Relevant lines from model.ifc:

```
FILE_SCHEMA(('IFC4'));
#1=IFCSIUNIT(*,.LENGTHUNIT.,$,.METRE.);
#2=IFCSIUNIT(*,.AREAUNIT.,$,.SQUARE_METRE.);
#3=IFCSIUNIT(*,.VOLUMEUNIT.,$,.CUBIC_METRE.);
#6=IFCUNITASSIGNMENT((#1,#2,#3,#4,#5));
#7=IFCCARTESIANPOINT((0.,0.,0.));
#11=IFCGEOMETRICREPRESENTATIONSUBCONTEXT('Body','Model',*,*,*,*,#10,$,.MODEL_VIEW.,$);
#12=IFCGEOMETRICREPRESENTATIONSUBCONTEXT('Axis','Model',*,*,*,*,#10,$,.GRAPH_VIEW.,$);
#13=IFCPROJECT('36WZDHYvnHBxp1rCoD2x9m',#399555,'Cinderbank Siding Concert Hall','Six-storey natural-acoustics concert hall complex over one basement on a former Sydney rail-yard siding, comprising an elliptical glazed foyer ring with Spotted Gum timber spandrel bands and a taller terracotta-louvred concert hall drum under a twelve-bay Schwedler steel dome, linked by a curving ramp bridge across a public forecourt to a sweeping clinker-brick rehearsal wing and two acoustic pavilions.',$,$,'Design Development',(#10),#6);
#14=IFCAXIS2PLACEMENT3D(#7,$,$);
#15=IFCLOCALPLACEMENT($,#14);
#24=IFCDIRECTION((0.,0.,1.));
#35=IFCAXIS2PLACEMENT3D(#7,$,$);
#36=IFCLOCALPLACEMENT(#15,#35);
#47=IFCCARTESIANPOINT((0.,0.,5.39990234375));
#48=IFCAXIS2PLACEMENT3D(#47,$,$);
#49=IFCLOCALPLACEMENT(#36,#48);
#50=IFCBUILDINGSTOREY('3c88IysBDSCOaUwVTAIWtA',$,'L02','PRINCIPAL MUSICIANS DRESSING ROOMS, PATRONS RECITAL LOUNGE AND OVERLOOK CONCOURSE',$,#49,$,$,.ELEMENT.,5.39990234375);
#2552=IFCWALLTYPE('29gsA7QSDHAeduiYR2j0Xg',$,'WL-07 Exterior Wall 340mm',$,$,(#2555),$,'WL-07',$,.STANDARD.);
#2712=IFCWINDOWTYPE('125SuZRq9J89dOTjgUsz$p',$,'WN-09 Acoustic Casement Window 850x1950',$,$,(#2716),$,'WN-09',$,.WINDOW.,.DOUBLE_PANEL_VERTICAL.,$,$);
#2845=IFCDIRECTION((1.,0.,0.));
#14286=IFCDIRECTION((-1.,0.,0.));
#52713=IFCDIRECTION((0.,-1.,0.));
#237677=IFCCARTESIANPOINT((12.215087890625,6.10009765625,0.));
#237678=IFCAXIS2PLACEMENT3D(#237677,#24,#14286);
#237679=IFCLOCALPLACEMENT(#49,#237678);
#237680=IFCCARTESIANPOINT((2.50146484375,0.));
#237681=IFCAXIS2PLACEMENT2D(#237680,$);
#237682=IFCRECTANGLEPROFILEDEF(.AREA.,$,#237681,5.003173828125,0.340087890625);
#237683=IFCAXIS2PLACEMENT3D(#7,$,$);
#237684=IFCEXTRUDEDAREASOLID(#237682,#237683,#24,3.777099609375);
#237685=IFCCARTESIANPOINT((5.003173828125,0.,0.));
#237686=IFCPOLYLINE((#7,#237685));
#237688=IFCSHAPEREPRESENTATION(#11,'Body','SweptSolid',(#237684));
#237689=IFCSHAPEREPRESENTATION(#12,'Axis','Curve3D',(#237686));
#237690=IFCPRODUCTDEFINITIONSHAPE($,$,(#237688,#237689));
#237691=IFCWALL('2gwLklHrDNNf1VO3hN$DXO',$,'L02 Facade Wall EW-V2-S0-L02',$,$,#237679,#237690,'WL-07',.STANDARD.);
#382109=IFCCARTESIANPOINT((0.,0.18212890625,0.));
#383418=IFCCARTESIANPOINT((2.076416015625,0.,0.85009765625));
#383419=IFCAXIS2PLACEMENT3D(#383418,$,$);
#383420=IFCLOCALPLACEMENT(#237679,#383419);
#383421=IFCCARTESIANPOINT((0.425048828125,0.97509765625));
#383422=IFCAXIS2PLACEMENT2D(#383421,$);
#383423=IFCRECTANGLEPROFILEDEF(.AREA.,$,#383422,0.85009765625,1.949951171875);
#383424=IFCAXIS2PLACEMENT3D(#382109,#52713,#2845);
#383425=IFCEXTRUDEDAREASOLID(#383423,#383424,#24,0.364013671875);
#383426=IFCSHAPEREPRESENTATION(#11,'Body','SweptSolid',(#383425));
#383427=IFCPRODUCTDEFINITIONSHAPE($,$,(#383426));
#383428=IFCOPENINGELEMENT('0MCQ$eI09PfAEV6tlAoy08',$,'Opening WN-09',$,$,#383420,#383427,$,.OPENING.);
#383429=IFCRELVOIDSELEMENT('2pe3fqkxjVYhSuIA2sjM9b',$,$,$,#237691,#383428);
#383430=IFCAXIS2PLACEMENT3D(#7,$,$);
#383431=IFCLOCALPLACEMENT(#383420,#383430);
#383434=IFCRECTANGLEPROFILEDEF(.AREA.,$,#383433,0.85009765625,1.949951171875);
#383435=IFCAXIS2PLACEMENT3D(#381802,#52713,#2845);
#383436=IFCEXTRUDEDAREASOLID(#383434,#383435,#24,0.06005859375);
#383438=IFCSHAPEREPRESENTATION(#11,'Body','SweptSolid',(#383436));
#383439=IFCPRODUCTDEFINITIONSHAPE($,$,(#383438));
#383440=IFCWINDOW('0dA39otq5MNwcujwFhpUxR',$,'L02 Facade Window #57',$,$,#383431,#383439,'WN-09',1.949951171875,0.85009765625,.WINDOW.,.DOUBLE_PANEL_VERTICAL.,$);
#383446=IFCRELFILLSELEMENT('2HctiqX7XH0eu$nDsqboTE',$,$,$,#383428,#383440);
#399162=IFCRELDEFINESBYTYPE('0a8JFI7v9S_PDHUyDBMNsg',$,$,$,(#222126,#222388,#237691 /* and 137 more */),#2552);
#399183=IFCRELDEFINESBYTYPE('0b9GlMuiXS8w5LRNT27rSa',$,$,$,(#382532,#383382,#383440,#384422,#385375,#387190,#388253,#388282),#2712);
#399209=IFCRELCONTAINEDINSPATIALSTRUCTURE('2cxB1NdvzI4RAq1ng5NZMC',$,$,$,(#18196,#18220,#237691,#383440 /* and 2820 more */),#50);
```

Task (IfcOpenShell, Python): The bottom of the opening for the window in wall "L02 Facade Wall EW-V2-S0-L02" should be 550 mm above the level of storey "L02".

```python
import numpy as np
import ifcopenshell
import ifcopenshell.api.geometry
import ifcopenshell.geom
import ifcopenshell.util.element
import ifcopenshell.util.placement
import ifcopenshell.util.shape
import ifcopenshell.util.unit

model = ifcopenshell.open("model.ifc")
unit_scale = ifcopenshell.util.unit.calculate_unit_scale(model)

window = model.by_guid("0dA39otq5MNwcujwFhpUxR")
opening = window.FillsVoids[0].RelatingOpeningElement
storey = ifcopenshell.util.element.get_container(window, ifc_class="IfcBuildingStorey")
level = ifcopenshell.util.placement.get_local_placement(storey.ObjectPlacement)[2, 3]

# The opening's origin need not be at the sill, so measure its lowest point.
shape = ifcopenshell.geom.create_shape(ifcopenshell.geom.settings(), opening)
bottom = ifcopenshell.util.shape.get_shape_bottom_elevation(shape, shape.geometry) / unit_scale
dz = level + 0.55 - bottom

shift = np.array([0.0, 0.0, dz])
# The window is placed relative to its opening, so it follows when the opening moves.
matrix = ifcopenshell.util.placement.get_local_placement(opening.ObjectPlacement)
matrix[:3, 3] += shift
ifcopenshell.api.geometry.edit_object_placement(
    model, product=opening, matrix=matrix, is_si=False, should_transform_children=True
)

print(f"moved by {dz * unit_scale:+.3f} m")

model.write("model_updated.ifc")
```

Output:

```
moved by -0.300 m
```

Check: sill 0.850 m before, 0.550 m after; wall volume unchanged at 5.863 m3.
